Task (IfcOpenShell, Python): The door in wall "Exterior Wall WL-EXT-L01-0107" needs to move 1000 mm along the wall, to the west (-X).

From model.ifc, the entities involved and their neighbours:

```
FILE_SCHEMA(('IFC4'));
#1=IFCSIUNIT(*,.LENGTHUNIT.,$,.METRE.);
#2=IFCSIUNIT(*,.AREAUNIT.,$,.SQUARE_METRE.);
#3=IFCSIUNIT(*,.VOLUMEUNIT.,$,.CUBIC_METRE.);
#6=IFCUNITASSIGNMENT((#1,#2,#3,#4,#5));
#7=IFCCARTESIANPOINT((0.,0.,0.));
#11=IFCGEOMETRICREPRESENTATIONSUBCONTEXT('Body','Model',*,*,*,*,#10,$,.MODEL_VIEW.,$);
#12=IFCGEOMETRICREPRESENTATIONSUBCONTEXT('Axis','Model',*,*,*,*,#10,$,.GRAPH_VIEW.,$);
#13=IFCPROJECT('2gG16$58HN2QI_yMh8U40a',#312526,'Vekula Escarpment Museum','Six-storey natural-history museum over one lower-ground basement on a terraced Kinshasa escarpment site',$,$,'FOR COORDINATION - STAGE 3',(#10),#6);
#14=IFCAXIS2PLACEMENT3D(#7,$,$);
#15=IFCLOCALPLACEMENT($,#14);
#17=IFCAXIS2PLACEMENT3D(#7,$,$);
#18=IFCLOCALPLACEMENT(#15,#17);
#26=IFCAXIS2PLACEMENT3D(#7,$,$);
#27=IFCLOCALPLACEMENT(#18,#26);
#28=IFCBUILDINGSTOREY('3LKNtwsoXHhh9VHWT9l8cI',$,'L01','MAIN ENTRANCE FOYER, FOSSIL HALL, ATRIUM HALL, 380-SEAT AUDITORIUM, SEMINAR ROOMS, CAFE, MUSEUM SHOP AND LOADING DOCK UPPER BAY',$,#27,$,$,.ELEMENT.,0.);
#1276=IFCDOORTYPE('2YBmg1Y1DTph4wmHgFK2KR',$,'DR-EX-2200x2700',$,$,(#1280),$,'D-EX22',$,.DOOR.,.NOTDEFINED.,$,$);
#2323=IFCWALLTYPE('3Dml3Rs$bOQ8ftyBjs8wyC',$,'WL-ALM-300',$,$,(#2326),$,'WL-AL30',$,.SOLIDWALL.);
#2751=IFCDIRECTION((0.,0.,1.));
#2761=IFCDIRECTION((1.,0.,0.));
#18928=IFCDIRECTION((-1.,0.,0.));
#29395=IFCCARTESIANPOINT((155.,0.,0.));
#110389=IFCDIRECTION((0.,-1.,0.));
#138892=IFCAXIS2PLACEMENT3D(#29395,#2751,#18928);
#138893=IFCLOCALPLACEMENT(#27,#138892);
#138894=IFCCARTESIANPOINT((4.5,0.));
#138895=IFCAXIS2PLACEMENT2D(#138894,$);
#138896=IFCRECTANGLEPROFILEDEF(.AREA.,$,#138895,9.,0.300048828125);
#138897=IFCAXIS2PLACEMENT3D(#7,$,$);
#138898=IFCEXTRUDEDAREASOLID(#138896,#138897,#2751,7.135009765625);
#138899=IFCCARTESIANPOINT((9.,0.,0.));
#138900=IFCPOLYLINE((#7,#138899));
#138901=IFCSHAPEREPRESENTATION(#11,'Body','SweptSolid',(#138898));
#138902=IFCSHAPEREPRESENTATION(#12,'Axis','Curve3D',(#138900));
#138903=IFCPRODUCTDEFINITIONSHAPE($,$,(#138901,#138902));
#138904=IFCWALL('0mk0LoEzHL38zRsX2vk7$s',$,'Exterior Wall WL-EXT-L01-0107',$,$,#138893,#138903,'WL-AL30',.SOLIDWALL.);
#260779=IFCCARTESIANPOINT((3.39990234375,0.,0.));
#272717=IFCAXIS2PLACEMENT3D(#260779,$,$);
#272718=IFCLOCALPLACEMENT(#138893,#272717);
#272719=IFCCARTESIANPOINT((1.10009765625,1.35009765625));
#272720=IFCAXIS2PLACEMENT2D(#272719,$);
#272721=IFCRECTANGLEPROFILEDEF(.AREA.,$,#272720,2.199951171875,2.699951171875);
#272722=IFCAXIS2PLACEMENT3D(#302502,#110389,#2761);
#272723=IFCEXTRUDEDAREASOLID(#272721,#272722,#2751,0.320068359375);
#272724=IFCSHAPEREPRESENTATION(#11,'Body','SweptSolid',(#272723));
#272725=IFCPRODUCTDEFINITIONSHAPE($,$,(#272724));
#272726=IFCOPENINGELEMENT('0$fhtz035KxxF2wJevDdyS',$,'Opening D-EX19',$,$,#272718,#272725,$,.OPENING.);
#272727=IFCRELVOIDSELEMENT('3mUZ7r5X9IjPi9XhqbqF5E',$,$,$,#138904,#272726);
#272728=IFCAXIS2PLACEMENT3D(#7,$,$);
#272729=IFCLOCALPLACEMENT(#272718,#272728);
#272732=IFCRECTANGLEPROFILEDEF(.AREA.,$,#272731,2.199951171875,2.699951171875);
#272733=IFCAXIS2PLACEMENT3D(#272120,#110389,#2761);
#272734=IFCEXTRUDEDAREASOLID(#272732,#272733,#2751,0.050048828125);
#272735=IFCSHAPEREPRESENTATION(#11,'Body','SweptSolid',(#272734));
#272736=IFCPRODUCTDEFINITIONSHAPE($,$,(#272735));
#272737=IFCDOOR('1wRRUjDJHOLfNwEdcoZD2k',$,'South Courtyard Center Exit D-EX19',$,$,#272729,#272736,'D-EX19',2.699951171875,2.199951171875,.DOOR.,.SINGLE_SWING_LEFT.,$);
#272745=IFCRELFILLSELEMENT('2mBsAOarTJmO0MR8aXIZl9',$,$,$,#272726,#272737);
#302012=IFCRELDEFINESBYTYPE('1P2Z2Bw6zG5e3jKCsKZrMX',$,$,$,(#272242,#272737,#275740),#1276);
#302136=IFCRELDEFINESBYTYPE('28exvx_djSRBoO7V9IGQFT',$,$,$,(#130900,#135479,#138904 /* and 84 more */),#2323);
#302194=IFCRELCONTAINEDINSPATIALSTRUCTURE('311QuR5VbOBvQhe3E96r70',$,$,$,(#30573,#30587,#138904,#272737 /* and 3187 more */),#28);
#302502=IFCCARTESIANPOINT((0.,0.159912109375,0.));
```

```python
import ifcopenshell
import ifcopenshell.api.geometry
import ifcopenshell.util.placement
import ifcopenshell.util.unit

model = ifcopenshell.open("model.ifc")
unit_scale = ifcopenshell.util.unit.calculate_unit_scale(model)

door = model.by_guid("1wRRUjDJHOLfNwEdcoZD2k")
opening = door.FillsVoids[0].RelatingOpeningElement
wall = opening.VoidsElements[0].RelatingBuildingElement

wall_matrix = ifcopenshell.util.placement.get_local_placement(wall.ObjectPlacement)
shift = wall_matrix[:3, 0] * 1 / unit_scale
before = ifcopenshell.util.placement.get_local_placement(door.ObjectPlacement)[:3, 3].copy()

# The door is placed relative to its opening, so it follows when the opening moves.
matrix = ifcopenshell.util.placement.get_local_placement(opening.ObjectPlacement)
matrix[:3, 3] += shift
ifcopenshell.api.geometry.edit_object_placement(
    model, product=opening, matrix=matrix, is_si=False, should_transform_children=True
)

after = ifcopenshell.util.placement.get_local_placement(door.ObjectPlacement)[:3, 3]
print("door moved by", (after - before).round(3) + 0.0)

model.write("model_edited.ifc")
```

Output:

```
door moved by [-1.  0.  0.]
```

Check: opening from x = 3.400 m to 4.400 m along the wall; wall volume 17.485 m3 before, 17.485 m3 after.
